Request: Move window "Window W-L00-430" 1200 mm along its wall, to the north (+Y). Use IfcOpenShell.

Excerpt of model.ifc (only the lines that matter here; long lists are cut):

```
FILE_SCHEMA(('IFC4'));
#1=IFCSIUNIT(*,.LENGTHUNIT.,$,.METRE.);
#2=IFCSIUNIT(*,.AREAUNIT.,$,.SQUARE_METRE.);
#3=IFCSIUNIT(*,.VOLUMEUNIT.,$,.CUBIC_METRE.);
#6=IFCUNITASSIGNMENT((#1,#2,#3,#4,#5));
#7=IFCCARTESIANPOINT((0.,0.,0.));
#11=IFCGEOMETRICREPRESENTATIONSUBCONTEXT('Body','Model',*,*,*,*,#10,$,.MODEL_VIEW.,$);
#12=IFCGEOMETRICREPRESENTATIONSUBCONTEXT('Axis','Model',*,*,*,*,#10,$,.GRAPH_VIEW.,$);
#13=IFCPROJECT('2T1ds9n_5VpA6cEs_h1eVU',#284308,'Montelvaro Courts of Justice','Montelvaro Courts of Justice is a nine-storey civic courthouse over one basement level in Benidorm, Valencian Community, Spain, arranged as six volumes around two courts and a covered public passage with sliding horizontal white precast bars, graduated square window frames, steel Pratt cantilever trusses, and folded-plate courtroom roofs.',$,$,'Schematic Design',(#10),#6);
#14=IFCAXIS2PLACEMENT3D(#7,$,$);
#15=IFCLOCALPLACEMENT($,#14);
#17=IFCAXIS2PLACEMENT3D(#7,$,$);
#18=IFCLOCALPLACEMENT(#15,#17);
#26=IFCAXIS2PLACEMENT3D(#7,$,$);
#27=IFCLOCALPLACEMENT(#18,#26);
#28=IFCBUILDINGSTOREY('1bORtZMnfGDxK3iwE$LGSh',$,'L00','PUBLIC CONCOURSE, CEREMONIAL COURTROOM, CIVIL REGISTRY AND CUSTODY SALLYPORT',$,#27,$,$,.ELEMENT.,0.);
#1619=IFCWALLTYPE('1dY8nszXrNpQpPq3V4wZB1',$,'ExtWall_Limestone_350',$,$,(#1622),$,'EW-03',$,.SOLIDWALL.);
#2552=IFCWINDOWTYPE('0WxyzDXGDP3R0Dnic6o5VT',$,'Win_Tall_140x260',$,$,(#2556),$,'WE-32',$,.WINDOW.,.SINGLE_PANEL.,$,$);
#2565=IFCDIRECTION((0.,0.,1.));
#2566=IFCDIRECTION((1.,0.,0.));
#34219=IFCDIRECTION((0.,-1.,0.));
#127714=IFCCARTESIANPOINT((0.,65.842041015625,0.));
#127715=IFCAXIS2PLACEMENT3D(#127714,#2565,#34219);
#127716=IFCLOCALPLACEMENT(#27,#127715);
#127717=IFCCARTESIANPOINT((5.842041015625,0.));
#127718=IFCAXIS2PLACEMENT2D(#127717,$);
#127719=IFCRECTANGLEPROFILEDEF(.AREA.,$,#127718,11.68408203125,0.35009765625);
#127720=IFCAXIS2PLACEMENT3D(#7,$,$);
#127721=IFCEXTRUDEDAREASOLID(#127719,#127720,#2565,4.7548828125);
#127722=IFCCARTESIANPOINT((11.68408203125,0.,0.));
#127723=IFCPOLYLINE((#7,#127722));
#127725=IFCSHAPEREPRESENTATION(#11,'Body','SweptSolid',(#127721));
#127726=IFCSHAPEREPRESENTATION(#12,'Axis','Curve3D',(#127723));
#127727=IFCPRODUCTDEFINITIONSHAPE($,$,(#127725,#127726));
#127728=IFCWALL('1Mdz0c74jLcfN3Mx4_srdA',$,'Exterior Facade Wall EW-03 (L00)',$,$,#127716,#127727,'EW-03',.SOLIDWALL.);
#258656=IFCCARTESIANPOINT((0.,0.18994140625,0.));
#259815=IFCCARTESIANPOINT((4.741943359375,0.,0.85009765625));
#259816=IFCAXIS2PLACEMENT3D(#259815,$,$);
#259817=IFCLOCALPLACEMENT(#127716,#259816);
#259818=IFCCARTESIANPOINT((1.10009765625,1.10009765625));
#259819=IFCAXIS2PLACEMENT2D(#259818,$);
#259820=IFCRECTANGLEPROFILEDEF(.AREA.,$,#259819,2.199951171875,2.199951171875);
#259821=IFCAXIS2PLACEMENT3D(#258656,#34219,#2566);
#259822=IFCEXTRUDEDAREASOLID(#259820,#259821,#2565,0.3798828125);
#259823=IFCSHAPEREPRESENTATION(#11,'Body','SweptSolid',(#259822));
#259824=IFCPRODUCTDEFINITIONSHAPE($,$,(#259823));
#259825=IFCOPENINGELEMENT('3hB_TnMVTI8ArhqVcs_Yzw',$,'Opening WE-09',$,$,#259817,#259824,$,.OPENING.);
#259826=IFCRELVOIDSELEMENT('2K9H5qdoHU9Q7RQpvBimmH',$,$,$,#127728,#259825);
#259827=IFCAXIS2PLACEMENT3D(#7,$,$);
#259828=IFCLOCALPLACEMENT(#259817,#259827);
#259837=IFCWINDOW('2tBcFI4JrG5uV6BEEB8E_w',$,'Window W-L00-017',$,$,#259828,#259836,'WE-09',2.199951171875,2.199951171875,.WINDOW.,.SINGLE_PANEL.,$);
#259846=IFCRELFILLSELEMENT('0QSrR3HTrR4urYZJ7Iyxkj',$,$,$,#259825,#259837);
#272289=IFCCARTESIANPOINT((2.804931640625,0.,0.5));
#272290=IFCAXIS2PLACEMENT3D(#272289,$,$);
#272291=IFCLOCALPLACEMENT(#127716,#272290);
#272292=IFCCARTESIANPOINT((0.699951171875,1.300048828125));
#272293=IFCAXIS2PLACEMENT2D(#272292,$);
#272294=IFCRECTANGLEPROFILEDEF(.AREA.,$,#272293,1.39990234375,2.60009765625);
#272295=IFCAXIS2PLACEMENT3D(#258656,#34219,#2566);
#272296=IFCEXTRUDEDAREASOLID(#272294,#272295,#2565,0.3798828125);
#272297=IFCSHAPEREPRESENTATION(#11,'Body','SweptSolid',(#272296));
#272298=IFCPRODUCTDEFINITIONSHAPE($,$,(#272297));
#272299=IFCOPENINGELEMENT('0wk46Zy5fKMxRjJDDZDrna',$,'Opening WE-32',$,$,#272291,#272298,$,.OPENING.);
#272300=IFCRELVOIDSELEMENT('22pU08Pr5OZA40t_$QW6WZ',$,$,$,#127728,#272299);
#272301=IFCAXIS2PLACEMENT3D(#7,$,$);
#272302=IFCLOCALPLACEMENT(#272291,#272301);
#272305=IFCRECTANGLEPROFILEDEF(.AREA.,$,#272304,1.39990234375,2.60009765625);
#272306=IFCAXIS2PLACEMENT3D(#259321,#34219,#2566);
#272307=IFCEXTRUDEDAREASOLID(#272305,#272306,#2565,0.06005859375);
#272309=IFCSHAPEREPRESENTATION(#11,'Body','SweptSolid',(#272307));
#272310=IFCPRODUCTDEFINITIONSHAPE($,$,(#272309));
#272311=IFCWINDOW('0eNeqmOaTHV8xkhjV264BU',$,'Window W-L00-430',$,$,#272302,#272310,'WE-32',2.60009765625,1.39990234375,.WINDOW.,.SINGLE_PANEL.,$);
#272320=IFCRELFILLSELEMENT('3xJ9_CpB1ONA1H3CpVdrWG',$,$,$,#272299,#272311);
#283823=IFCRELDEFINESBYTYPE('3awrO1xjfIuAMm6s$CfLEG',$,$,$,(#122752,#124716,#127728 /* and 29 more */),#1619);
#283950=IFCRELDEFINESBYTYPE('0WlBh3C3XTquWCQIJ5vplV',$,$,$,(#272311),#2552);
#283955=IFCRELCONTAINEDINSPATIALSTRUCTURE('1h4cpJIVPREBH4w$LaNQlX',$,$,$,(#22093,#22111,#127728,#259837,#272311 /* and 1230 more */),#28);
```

```python
import ifcopenshell
import ifcopenshell.api.geometry
import ifcopenshell.util.placement

model = ifcopenshell.open("model.ifc")

window = model.by_guid("0eNeqmOaTHV8xkhjV264BU")
opening = window.FillsVoids[0].RelatingOpeningElement
wall = opening.VoidsElements[0].RelatingBuildingElement

wall_matrix = ifcopenshell.util.placement.get_local_placement(wall.ObjectPlacement)
shift = wall_matrix[:3, 0] * -1.2
before = ifcopenshell.util.placement.get_local_placement(window.ObjectPlacement)[:3, 3].copy()

# The window is placed relative to its opening, so it follows when the opening moves.
matrix = ifcopenshell.util.placement.get_local_placement(opening.ObjectPlacement)
matrix[:3, 3] += shift
ifcopenshell.api.geometry.edit_object_placement(
    model, product=opening, matrix=matrix, is_si=False, should_transform_children=True
)

after = ifcopenshell.util.placement.get_local_placement(window.ObjectPlacement)[:3, 3]
print("window moved by", (after - before).round(3) + 0.0)

model.write("model-out.ifc")
```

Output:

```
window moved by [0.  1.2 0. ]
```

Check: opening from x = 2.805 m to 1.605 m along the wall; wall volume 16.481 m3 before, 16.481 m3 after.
